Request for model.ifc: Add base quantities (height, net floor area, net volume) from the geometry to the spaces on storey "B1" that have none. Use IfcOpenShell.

First a look at what the model holds.

```python
import ifcopenshell
import ifcopenshell.util.element
import ifcopenshell.util.unit

model = ifcopenshell.open("model.ifc")
print(model.schema)
for unit_type in ("LENGTHUNIT", "AREAUNIT", "VOLUMEUNIT"):
    print(unit_type, ifcopenshell.util.unit.calculate_unit_scale(model, unit_type))
storey = next(s for s in model.by_type("IfcBuildingStorey") if s.Name == "B1")
spaces = [e for e in ifcopenshell.util.element.get_decomposition(storey) if e.is_a("IfcSpace")]
for e in sorted(spaces, key=lambda e: e.id()):
    print(e.id(), e.is_a(), e.Name, list(ifcopenshell.util.element.get_psets(e, qtos_only=True)), sep=" | ")
```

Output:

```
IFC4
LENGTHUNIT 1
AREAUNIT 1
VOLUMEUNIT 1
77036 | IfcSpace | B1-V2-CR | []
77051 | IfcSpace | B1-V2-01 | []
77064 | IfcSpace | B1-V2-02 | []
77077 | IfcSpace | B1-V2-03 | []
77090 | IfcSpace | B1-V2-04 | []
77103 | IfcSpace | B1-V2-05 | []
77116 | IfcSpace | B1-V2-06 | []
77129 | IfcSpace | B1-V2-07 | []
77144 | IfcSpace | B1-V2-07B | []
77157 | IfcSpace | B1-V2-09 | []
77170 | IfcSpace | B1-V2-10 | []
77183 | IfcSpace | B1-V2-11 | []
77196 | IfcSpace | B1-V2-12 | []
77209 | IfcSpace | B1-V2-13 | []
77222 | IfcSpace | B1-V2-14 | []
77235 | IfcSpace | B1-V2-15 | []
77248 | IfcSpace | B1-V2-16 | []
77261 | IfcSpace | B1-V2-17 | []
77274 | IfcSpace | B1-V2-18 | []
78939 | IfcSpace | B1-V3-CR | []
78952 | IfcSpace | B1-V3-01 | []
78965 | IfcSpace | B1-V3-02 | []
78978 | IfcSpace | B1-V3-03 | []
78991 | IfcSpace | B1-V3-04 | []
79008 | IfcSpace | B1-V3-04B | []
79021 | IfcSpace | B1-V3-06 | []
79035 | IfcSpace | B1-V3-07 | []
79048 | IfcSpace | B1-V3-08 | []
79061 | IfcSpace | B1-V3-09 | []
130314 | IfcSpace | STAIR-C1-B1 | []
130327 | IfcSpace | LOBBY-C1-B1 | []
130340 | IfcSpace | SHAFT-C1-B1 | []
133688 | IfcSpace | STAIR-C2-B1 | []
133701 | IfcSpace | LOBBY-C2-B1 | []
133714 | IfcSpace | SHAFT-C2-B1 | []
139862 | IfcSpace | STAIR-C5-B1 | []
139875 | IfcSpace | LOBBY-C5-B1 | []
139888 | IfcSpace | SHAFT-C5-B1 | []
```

```python
import ifcopenshell
import ifcopenshell.api.pset
import ifcopenshell.geom
import ifcopenshell.util.element
import ifcopenshell.util.shape
import ifcopenshell.util.unit

model = ifcopenshell.open("model.ifc")
unit_scale = ifcopenshell.util.unit.calculate_unit_scale(model)
area_scale = ifcopenshell.util.unit.calculate_unit_scale(model, "AREAUNIT")
volume_scale = ifcopenshell.util.unit.calculate_unit_scale(model, "VOLUMEUNIT")
settings = ifcopenshell.geom.settings()

storey = next(s for s in model.by_type("IfcBuildingStorey") if s.Name == "B1")
spaces = [e for e in ifcopenshell.util.element.get_decomposition(storey) if e.is_a("IfcSpace")]

for e in sorted(spaces, key=lambda e: e.id()):
    if ifcopenshell.util.element.get_psets(e, qtos_only=True, should_inherit=False):
        continue
    # Geometry comes back in metres, in the element's own axes.
    shape = ifcopenshell.geom.create_shape(settings, e)
    values = {
        "Height": ifcopenshell.util.shape.get_z(shape.geometry) / unit_scale,
        "NetFloorArea": ifcopenshell.util.shape.get_footprint_area(shape.geometry) / area_scale,
        "NetVolume": ifcopenshell.util.shape.get_volume(shape.geometry) / volume_scale,
    }
    qto = ifcopenshell.api.pset.add_qto(model, product=e, name="Qto_SpaceBaseQuantities")
    ifcopenshell.api.pset.edit_qto(model, qto=qto, properties=values)
    print(e.id(), {k: round(v, 3) for k, v in values.items()})

model.write("model_updated.ifc")
```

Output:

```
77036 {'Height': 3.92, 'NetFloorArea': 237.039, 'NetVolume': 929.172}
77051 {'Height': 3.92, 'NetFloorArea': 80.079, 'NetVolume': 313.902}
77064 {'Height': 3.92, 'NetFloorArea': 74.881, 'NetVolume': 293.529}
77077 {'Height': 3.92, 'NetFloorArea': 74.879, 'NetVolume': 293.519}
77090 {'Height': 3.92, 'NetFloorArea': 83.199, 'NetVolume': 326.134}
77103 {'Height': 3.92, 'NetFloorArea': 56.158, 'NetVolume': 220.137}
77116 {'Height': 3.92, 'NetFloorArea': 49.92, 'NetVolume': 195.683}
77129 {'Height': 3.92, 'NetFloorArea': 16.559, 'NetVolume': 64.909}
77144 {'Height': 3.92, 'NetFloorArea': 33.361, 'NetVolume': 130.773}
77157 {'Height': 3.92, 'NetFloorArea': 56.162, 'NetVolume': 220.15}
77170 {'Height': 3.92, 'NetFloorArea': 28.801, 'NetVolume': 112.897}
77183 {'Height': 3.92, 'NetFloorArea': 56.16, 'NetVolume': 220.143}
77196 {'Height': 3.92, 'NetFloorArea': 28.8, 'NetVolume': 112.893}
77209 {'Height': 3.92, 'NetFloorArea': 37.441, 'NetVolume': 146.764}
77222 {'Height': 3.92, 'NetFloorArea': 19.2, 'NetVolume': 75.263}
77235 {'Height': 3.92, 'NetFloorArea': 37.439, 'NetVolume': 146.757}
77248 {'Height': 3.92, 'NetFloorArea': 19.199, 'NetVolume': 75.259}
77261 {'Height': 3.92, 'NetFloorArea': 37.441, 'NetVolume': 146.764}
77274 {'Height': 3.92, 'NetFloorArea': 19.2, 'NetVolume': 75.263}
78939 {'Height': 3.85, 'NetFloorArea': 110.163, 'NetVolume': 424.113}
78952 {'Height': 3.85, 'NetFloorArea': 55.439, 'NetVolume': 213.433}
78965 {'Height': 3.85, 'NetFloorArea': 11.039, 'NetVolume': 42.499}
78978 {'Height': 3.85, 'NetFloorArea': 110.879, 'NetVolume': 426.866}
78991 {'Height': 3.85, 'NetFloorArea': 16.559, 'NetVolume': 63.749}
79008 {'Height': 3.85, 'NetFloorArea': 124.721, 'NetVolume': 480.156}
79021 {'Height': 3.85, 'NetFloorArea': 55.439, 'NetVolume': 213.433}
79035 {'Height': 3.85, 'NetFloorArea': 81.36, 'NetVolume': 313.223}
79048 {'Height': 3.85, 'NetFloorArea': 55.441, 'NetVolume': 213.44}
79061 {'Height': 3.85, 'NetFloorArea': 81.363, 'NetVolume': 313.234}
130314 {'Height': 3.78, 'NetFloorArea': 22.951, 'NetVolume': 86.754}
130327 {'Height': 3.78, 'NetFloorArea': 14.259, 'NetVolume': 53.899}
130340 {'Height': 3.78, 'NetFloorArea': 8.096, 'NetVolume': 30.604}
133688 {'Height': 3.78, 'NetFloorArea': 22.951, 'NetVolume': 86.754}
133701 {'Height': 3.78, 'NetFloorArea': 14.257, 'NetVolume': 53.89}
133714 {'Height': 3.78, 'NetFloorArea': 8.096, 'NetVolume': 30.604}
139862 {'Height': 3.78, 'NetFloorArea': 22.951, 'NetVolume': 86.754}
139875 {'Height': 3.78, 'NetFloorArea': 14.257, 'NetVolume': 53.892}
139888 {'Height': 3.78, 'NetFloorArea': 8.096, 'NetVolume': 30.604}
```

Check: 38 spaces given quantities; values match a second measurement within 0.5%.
